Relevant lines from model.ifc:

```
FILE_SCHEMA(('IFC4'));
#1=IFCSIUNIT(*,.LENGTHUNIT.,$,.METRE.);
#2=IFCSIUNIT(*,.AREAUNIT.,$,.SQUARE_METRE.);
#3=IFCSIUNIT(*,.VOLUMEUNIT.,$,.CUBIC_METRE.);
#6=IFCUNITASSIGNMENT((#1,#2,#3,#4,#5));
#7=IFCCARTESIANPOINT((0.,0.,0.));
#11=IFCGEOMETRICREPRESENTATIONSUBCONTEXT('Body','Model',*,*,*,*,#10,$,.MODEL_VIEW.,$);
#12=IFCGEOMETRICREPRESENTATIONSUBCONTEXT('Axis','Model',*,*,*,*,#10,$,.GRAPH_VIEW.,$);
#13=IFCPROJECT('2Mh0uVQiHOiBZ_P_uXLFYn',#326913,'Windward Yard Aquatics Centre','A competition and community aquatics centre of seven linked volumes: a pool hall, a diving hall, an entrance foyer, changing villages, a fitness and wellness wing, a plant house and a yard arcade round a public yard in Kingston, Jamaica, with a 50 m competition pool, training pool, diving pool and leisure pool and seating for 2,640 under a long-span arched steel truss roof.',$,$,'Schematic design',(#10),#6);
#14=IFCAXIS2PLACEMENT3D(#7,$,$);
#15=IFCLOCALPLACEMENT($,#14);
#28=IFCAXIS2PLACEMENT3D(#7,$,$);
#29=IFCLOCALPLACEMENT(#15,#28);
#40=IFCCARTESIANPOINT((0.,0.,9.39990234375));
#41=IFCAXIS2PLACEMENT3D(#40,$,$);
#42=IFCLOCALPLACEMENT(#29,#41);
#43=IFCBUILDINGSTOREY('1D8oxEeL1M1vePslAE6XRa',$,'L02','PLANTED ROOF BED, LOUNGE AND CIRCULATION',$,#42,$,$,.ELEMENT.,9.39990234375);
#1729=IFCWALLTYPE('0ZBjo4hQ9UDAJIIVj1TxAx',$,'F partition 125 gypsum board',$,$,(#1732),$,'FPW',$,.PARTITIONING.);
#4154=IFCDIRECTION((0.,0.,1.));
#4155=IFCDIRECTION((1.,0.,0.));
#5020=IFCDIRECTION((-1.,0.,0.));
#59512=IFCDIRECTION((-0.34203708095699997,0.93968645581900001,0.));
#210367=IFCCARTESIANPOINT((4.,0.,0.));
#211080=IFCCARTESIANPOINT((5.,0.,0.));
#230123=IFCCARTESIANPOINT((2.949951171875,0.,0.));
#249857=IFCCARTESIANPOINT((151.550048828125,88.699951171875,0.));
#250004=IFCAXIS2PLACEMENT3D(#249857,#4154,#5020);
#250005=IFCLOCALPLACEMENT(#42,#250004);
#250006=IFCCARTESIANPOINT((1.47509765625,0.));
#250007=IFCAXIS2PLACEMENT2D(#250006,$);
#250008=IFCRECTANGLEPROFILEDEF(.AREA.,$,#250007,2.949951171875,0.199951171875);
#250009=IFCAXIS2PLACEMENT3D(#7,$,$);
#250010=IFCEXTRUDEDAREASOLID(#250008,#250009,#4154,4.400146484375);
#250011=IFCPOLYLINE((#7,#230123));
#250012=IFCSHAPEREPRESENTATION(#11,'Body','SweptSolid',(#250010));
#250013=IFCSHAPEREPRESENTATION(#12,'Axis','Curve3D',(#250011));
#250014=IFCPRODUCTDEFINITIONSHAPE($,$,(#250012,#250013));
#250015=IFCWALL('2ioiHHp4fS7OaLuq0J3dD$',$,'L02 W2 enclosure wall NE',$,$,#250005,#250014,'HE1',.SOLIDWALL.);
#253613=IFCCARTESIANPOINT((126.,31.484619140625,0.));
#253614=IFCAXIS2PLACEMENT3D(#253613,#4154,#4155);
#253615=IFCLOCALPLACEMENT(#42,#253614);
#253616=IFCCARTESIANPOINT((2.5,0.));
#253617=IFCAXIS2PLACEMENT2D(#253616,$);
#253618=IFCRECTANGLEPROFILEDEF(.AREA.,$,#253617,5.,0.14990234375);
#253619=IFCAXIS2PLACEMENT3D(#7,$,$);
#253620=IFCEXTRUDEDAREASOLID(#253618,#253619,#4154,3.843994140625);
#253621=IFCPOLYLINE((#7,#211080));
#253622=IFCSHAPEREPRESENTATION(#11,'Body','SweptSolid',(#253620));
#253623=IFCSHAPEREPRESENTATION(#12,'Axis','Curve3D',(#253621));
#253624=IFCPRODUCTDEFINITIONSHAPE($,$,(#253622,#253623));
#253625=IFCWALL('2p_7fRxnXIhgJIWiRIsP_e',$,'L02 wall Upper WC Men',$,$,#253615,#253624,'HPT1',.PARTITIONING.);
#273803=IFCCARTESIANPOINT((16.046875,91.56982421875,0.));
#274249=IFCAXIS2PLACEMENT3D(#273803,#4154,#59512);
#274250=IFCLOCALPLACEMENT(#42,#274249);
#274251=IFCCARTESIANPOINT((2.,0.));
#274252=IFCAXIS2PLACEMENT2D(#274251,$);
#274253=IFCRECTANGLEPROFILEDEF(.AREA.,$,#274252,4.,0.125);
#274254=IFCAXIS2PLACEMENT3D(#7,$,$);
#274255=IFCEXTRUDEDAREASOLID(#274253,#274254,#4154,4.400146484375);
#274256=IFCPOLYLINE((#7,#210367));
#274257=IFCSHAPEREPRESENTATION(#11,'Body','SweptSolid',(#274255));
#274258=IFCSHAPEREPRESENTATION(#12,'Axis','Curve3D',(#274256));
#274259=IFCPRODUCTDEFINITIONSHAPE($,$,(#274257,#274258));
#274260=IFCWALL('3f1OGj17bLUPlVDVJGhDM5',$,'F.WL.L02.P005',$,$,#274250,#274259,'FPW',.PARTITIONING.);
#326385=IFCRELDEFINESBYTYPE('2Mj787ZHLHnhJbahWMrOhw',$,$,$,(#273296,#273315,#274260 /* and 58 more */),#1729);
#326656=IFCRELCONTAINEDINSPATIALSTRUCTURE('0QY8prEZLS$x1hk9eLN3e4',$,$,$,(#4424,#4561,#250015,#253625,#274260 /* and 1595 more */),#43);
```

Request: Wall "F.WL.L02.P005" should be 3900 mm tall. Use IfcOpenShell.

```python
import ifcopenshell
import ifcopenshell.geom
import ifcopenshell.util.representation
import ifcopenshell.util.shape

model = ifcopenshell.open("model.ifc")
settings = ifcopenshell.geom.settings()


def volume(element):
    """Net volume in cubic metres, openings subtracted."""
    shape = ifcopenshell.geom.create_shape(settings, element)
    return ifcopenshell.util.shape.get_volume(shape.geometry)


wall = model.by_guid("3f1OGj17bLUPlVDVJGhDM5")
before = volume(wall)

body = ifcopenshell.util.representation.get_representation(wall, "Model", "Body")
solid = body.Items[0]
old_height = solid.Depth
solid.Depth = 3.9
after = volume(wall)

print(f"height {old_height:g} -> {solid.Depth:g}, volume {before:.3f} -> {after:.3f} m3")

model.write("model_v2.ifc")
```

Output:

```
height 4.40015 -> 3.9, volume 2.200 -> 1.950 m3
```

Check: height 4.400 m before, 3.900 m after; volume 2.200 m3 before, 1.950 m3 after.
